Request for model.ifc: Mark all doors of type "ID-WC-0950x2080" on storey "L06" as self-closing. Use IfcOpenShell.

First a look at what the model holds.

```python
import ifcopenshell
import ifcopenshell.util.element

model = ifcopenshell.open("model.ifc")
print(model.schema)
storey = next(s for s in model.by_type("IfcBuildingStorey") if s.Name == "L06")
doors = [e for e in ifcopenshell.util.element.get_decomposition(storey) if e.is_a("IfcDoor")]
seen = {}
for e in doors:
    element_type = ifcopenshell.util.element.get_type(e)
    key = (element_type.Name if element_type != e and element_type else None, ifcopenshell.util.element.get_pset(e, "Pset_DoorCommon", "SelfClosing"))
    seen[key] = seen.get(key, 0) + 1
for (name, value), count in sorted(seen.items(), key=str):
    print(count, "x", name, "|", value)
```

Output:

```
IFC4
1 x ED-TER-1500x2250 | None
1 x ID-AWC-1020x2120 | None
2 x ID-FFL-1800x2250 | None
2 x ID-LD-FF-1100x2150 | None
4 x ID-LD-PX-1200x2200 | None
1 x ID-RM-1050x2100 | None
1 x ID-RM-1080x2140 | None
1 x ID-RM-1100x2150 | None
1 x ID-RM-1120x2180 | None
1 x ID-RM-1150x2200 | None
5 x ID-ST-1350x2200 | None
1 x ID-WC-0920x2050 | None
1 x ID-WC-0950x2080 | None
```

```python
import ifcopenshell
import ifcopenshell.api.pset
import ifcopenshell.util.element

model = ifcopenshell.open("model.ifc")

storey = next(s for s in model.by_type("IfcBuildingStorey") if s.Name == "L06")
doors = [e for e in ifcopenshell.util.element.get_decomposition(storey) if e.is_a("IfcDoor")]

count = 0
for e in doors:
    element_type = ifcopenshell.util.element.get_type(e)
    if element_type in (None, e) or element_type.Name != "ID-WC-0950x2080":
        continue
    # add_pset returns the element's existing set when there is one.
    pset = ifcopenshell.api.pset.add_pset(model, product=e, name="Pset_DoorCommon")
    ifcopenshell.api.pset.edit_pset(model, pset=pset, properties={"SelfClosing": True})
    count += 1

print(count, "doors updated")

model.write("model-out.ifc")
```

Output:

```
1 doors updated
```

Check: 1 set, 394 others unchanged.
